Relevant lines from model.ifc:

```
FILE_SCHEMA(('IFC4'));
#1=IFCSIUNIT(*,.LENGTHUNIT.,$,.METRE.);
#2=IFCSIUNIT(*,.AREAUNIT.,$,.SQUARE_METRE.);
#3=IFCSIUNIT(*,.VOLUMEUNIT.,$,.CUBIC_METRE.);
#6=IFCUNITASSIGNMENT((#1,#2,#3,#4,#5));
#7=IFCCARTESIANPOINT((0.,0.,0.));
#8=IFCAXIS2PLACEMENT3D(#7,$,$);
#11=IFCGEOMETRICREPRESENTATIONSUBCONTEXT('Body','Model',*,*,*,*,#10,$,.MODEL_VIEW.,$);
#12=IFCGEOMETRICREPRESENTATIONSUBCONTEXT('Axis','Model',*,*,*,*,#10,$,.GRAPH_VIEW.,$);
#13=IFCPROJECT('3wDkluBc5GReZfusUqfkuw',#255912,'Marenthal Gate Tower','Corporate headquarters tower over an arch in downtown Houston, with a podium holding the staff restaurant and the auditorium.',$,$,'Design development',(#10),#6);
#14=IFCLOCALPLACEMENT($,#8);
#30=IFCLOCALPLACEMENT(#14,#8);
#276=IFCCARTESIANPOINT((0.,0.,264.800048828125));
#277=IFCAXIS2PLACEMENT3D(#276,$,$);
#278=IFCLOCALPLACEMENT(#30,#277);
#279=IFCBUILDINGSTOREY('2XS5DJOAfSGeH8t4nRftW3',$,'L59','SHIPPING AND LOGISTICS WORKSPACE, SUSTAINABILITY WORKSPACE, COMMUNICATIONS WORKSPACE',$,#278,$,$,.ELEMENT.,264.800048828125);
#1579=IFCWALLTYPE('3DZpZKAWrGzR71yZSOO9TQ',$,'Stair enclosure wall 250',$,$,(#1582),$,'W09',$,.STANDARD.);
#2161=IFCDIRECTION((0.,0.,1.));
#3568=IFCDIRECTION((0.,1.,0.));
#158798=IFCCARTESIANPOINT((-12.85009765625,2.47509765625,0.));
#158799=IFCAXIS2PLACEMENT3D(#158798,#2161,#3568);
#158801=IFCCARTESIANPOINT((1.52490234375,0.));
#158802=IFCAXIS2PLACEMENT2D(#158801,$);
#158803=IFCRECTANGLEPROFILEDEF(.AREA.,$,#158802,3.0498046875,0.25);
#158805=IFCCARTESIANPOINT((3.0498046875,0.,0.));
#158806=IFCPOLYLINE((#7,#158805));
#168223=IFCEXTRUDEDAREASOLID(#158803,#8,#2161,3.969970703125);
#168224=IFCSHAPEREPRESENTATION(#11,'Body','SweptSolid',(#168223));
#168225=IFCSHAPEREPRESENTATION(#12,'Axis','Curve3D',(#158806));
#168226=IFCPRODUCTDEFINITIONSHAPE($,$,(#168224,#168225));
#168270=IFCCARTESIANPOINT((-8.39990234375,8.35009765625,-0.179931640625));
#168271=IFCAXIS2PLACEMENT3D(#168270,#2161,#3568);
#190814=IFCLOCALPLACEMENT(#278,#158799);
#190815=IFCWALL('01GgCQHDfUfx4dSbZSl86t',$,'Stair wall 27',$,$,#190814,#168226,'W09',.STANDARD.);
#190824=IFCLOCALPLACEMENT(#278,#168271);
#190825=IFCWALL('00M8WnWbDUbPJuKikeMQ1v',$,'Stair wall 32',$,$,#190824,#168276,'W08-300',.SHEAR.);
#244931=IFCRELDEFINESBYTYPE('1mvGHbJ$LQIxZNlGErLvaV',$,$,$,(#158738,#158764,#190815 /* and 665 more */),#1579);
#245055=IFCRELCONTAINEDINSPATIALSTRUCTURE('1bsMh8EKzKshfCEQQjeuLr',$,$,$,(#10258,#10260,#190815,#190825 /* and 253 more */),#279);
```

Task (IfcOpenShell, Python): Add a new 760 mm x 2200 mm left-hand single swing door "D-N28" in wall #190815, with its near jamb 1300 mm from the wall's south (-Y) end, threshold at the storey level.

```python
import numpy as np
import ifcopenshell
import ifcopenshell.api.feature
import ifcopenshell.api.geometry
import ifcopenshell.api.root
import ifcopenshell.api.spatial
import ifcopenshell.geom
import ifcopenshell.util.element
import ifcopenshell.util.placement
import ifcopenshell.util.representation
import ifcopenshell.util.shape
import ifcopenshell.util.unit

model = ifcopenshell.open("model.ifc")
unit_scale = ifcopenshell.util.unit.calculate_unit_scale(model)
settings = ifcopenshell.geom.settings()


def volume(element):
    """Net volume in cubic metres, openings subtracted."""
    shape = ifcopenshell.geom.create_shape(settings, element)
    return ifcopenshell.util.shape.get_volume(shape.geometry)


wall = model.by_guid("01GgCQHDfUfx4dSbZSl86t")
storey = ifcopenshell.util.element.get_container(wall, ifc_class="IfcBuildingStorey")
context = ifcopenshell.util.representation.get_context(model, "Model", "Body", "MODEL_VIEW")
before = volume(wall)

width, height, from_end, sill = 0.76, 2.2, 1.3, 0.0  # metres

# The wall runs along its own X axis, and the end named is its -X end.
wall_shape = ifcopenshell.geom.create_shape(settings, wall)
x, y, z = ifcopenshell.util.shape.get_vertices(wall_shape.geometry).T
start = x.min() + from_end
face, thickness = float(y.min()), float(y.max() - y.min())
wall_matrix = ifcopenshell.util.placement.get_local_placement(wall.ObjectPlacement)
level = ifcopenshell.util.placement.get_local_placement(storey.ObjectPlacement)[2, 3]


def in_wall(x, y):
    """Placement at x, y metres in the wall's axes, at sill height."""
    matrix = wall_matrix.copy()
    matrix[:, 3] = wall_matrix @ np.array([x / unit_scale, y / unit_scale, 0.0, 1.0])
    matrix[2, 3] = level + sill / unit_scale
    return matrix


# Opening: a box that overshoots both wall faces by 50 mm.
opening = ifcopenshell.api.root.create_entity(model, ifc_class="IfcOpeningElement", predefined_type="OPENING")
box = ifcopenshell.api.geometry.add_wall_representation(
    model, context=context, length=width, height=height, thickness=thickness + 0.1
)
ifcopenshell.api.geometry.assign_representation(model, product=opening, representation=box)
ifcopenshell.api.geometry.edit_object_placement(model, product=opening, matrix=in_wall(start, face - 0.05), is_si=False)
ifcopenshell.api.feature.add_feature(model, feature=opening, element=wall)

door = ifcopenshell.api.root.create_entity(model, ifc_class="IfcDoor", name="D-N28", predefined_type="DOOR")
door.OverallWidth, door.OverallHeight = width / unit_scale, height / unit_scale
door.OperationType = "SINGLE_SWING_LEFT"
body = ifcopenshell.api.geometry.add_door_representation(
    model,
    context=context,
    overall_width=door.OverallWidth,
    overall_height=door.OverallHeight,
    operation_type="SINGLE_SWING_LEFT",
    lining_properties={"LiningDepth": thickness / unit_scale, "ThresholdDepth": thickness / unit_scale},
)
ifcopenshell.api.geometry.assign_representation(model, product=door, representation=body)
ifcopenshell.api.spatial.assign_container(model, products=[door], relating_structure=storey)
ifcopenshell.api.feature.add_filling(model, opening=opening, element=door)

# The lining spans the wall, so the door starts at the wall face.
ifcopenshell.api.geometry.edit_object_placement(model, product=door, matrix=in_wall(start, face), is_si=False)

after = volume(wall)

print(f"wall volume {before:.3f} -> {after:.3f} m3")

model.write("model_updated.ifc")
```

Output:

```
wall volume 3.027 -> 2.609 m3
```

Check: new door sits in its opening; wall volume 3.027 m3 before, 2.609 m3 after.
